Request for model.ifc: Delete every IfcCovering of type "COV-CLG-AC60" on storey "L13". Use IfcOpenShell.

First a look at what the model holds.

```python
import ifcopenshell
import ifcopenshell.util.element

model = ifcopenshell.open("model.ifc")
print(model.schema)
storey = next(s for s in model.by_type("IfcBuildingStorey") if s.Name == "L13")
coverings = [e for e in ifcopenshell.util.element.get_decomposition(storey) if e.is_a("IfcCovering")]
seen = {}
for e in coverings:
    element_type = ifcopenshell.util.element.get_type(e)
    name = element_type.Name if element_type not in (None, e) else None
    seen[name] = seen.get(name, 0) + 1
for name, count in sorted(seen.items(), key=str):
    print(count, "x", name)
```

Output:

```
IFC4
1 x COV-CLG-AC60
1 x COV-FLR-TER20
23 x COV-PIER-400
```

```python
import ifcopenshell
import ifcopenshell.api.root
import ifcopenshell.util.element

model = ifcopenshell.open("model.ifc")

storey = next(s for s in model.by_type("IfcBuildingStorey") if s.Name == "L13")
coverings = [e for e in ifcopenshell.util.element.get_decomposition(storey) if e.is_a("IfcCovering")]
targets = [e for e in coverings if (t := ifcopenshell.util.element.get_type(e)) not in (None, e) and t.Name == "COV-CLG-AC60"]

for e in targets:
    ifcopenshell.api.root.remove_product(model, product=e)
print(len(targets), "removed")

model.write("model_updated.ifc")
```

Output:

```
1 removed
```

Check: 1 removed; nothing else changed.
